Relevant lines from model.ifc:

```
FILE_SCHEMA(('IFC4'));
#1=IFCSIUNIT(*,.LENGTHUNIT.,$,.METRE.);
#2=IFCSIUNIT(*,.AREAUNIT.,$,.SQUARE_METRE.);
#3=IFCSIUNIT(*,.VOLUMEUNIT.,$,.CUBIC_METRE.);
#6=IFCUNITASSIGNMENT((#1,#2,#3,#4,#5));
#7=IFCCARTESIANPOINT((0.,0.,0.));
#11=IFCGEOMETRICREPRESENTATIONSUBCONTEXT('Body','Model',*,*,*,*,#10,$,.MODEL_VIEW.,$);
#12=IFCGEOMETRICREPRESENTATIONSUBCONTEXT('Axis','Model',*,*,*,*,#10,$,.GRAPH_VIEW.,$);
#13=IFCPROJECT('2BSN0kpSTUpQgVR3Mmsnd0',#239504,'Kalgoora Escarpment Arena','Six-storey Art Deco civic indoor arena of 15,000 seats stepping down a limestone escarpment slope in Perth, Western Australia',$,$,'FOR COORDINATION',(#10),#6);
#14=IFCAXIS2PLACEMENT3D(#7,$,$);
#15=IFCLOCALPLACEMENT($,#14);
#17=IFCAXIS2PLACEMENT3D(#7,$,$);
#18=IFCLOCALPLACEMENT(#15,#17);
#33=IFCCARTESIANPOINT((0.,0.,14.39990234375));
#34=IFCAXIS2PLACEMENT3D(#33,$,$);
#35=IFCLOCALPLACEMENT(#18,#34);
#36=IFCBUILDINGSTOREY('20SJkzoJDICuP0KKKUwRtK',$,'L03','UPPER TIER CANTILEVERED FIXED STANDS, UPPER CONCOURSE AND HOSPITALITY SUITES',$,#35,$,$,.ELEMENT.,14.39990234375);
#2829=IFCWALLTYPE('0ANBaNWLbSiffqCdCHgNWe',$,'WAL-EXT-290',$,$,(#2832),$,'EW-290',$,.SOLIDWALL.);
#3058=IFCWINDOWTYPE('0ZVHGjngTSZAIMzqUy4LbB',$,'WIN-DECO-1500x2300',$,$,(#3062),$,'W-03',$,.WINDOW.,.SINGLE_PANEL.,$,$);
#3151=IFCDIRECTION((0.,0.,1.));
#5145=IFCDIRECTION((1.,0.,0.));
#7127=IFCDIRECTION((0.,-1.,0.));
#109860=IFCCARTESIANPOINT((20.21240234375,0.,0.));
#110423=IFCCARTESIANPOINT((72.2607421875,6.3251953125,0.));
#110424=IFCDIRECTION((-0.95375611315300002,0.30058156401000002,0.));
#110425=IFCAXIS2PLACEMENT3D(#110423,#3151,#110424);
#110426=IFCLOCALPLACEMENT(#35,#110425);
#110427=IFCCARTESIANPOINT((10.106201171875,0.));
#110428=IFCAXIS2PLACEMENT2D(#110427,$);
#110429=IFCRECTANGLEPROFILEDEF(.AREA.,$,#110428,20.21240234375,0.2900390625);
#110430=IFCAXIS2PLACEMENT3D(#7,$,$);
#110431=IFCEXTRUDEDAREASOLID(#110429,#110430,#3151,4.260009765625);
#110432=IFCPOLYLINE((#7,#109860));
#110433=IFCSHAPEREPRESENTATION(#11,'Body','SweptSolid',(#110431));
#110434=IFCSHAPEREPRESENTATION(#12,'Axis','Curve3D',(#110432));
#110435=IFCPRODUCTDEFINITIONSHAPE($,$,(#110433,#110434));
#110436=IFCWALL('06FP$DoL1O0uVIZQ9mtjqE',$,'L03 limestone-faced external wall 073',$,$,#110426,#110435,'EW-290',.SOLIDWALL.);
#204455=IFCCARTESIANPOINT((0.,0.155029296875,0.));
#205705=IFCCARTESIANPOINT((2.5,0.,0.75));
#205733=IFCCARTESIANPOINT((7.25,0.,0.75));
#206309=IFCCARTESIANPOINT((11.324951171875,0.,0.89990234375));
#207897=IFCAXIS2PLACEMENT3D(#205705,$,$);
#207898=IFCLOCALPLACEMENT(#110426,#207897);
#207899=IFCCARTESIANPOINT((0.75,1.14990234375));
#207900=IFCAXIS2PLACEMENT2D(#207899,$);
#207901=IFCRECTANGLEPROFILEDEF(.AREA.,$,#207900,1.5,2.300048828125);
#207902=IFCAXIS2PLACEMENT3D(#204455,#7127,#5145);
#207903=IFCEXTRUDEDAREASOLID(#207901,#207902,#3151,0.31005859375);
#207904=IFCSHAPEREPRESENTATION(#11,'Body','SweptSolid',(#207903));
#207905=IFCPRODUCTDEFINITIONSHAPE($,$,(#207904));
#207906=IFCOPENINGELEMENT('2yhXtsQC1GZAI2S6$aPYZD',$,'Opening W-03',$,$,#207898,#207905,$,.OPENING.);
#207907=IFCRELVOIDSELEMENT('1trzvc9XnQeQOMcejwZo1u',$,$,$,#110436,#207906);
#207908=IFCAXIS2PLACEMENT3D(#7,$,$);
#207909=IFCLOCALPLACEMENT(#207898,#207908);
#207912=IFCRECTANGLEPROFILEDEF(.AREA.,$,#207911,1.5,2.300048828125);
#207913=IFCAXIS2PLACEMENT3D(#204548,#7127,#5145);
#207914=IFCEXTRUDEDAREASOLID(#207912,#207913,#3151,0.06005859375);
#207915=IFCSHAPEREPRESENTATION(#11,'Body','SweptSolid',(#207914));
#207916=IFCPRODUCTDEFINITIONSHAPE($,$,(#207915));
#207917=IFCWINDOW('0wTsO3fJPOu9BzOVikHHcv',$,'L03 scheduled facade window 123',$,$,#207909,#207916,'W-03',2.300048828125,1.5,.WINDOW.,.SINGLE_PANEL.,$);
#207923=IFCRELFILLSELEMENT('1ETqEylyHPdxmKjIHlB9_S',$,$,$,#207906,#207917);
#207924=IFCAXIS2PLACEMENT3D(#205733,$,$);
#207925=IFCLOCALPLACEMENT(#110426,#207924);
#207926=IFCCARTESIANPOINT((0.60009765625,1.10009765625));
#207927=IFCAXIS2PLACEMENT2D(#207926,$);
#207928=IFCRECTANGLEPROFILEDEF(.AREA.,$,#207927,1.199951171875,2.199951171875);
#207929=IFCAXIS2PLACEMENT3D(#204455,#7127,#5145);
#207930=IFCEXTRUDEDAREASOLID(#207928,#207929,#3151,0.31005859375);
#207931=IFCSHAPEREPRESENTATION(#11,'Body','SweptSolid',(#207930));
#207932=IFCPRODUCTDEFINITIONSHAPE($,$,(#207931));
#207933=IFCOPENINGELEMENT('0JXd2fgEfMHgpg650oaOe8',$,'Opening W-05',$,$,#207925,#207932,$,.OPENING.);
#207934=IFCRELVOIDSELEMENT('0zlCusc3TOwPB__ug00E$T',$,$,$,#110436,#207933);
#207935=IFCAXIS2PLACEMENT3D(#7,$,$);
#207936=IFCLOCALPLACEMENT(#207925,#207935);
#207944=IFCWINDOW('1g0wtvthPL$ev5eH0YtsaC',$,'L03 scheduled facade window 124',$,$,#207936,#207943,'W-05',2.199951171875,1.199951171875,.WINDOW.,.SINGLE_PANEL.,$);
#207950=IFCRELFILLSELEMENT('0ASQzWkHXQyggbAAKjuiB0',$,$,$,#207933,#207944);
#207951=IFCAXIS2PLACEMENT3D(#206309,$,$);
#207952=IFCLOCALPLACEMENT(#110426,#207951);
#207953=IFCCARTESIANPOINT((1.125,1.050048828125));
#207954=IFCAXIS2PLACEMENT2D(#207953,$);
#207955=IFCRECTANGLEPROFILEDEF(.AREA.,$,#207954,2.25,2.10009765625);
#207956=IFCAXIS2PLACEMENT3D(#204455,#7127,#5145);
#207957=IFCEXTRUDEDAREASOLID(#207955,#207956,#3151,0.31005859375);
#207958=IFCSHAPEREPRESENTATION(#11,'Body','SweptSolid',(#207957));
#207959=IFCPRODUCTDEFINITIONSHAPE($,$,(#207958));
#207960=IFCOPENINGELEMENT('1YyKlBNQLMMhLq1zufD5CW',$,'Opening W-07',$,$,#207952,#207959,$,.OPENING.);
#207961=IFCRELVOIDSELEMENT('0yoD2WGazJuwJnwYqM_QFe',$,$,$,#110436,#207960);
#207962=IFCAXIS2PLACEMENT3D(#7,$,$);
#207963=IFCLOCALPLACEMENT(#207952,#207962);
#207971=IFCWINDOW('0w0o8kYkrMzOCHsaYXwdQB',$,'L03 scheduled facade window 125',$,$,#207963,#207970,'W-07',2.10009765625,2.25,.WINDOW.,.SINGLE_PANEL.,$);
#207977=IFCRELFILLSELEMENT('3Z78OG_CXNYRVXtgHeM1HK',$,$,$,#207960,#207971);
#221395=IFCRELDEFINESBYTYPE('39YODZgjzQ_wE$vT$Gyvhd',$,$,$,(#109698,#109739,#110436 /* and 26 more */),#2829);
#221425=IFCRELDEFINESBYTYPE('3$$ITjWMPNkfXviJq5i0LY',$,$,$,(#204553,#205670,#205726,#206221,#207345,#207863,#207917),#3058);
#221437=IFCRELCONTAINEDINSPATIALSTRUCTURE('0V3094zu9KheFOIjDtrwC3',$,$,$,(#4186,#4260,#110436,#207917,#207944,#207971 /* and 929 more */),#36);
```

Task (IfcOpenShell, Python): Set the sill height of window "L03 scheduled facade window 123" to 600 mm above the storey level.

```python
import numpy as np
import ifcopenshell
import ifcopenshell.api.geometry
import ifcopenshell.geom
import ifcopenshell.util.element
import ifcopenshell.util.placement
import ifcopenshell.util.shape
import ifcopenshell.util.unit

model = ifcopenshell.open("model.ifc")
unit_scale = ifcopenshell.util.unit.calculate_unit_scale(model)

window = model.by_guid("0wTsO3fJPOu9BzOVikHHcv")
opening = window.FillsVoids[0].RelatingOpeningElement
storey = ifcopenshell.util.element.get_container(window, ifc_class="IfcBuildingStorey")
level = ifcopenshell.util.placement.get_local_placement(storey.ObjectPlacement)[2, 3]

# The opening's origin need not be at the sill, so measure its lowest point.
shape = ifcopenshell.geom.create_shape(ifcopenshell.geom.settings(), opening)
bottom = ifcopenshell.util.shape.get_shape_bottom_elevation(shape, shape.geometry) / unit_scale
dz = level + 0.6 - bottom

shift = np.array([0.0, 0.0, dz])
# The window is placed relative to its opening, so it follows when the opening moves.
matrix = ifcopenshell.util.placement.get_local_placement(opening.ObjectPlacement)
matrix[:3, 3] += shift
ifcopenshell.api.geometry.edit_object_placement(
    model, product=opening, matrix=matrix, is_si=False, should_transform_children=True
)

print(f"moved by {dz * unit_scale:+.3f} m")

model.write("model_updated.ifc")
```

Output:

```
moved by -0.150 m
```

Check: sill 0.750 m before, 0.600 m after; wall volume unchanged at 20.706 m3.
